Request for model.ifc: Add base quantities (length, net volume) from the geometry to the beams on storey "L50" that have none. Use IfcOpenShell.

First a look at what the model holds.

```python
import ifcopenshell
import ifcopenshell.util.element
import ifcopenshell.util.unit

model = ifcopenshell.open("model.ifc")
print(model.schema)
for unit_type in ("LENGTHUNIT", "AREAUNIT", "VOLUMEUNIT"):
    print(unit_type, ifcopenshell.util.unit.calculate_unit_scale(model, unit_type))
storey = next(s for s in model.by_type("IfcBuildingStorey") if s.Name == "L50")
beams = [e for e in ifcopenshell.util.element.get_decomposition(storey) if e.is_a("IfcBeam")]
for e in sorted(beams, key=lambda e: e.id()):
    print(e.id(), e.is_a(), e.Name, list(ifcopenshell.util.element.get_psets(e, qtos_only=True)), sep=" | ")
```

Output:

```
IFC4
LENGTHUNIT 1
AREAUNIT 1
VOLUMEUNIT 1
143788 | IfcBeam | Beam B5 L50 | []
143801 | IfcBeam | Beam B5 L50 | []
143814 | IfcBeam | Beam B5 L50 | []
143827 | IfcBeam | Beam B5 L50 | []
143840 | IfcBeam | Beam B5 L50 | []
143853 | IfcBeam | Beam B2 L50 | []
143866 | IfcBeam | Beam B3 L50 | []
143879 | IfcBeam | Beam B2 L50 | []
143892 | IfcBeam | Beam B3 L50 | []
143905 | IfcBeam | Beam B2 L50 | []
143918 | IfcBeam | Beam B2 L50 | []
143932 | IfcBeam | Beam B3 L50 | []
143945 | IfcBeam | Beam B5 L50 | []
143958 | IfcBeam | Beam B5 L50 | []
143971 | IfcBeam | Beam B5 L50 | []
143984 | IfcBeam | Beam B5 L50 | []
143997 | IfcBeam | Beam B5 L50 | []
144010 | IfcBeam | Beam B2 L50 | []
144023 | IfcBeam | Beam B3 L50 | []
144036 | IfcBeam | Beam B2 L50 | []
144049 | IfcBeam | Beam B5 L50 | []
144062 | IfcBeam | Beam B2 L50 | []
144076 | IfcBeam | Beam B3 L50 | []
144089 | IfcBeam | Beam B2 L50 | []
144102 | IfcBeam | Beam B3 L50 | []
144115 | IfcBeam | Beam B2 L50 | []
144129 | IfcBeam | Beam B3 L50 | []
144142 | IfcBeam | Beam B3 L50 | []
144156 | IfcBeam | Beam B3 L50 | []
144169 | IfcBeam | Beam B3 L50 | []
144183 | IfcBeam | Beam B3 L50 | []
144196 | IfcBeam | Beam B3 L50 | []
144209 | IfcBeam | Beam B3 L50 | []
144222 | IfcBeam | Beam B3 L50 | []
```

```python
import ifcopenshell
import ifcopenshell.api.pset
import ifcopenshell.geom
import ifcopenshell.util.element
import ifcopenshell.util.shape
import ifcopenshell.util.unit

model = ifcopenshell.open("model.ifc")
unit_scale = ifcopenshell.util.unit.calculate_unit_scale(model)
volume_scale = ifcopenshell.util.unit.calculate_unit_scale(model, "VOLUMEUNIT")
settings = ifcopenshell.geom.settings()

storey = next(s for s in model.by_type("IfcBuildingStorey") if s.Name == "L50")
beams = [e for e in ifcopenshell.util.element.get_decomposition(storey) if e.is_a("IfcBeam")]

for e in sorted(beams, key=lambda e: e.id()):
    if ifcopenshell.util.element.get_psets(e, qtos_only=True, should_inherit=False):
        continue
    # Geometry comes back in metres, in the element's own axes.
    shape = ifcopenshell.geom.create_shape(settings, e)
    values = {
        "Length": ifcopenshell.util.shape.get_max_xyz(shape.geometry) / unit_scale,
        "NetVolume": ifcopenshell.util.shape.get_volume(shape.geometry) / volume_scale,
    }
    qto = ifcopenshell.api.pset.add_qto(model, product=e, name="Qto_BeamBaseQuantities")
    ifcopenshell.api.pset.edit_qto(model, qto=qto, properties=values)
    print(e.id(), {k: round(v, 3) for k, v in values.items()})

model.write("model_edited.ifc")
```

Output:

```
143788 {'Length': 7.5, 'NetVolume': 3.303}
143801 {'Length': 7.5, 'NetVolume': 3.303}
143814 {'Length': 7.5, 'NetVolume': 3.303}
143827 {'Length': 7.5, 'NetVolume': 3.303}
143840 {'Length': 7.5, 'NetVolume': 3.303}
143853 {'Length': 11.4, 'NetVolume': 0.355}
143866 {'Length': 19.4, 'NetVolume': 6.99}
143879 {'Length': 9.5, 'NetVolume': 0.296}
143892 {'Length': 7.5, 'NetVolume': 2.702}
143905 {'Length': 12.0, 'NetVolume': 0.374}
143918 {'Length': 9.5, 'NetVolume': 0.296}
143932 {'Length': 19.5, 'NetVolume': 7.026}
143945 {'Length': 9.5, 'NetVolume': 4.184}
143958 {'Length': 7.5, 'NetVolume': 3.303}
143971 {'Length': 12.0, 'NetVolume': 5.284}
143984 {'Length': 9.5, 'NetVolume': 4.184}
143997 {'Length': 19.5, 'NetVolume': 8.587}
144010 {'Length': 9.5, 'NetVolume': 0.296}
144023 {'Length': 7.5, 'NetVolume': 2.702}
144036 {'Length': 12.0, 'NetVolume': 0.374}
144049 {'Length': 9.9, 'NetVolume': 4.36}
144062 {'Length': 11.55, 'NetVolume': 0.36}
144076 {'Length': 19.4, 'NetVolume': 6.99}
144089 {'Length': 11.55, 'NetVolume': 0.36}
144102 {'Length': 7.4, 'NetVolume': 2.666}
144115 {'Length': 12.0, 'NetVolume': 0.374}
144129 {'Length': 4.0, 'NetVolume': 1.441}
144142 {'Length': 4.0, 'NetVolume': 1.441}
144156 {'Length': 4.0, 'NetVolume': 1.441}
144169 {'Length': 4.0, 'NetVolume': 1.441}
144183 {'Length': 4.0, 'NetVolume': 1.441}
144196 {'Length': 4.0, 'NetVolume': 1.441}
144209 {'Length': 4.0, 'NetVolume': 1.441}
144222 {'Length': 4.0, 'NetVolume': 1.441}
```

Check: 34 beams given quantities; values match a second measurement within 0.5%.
